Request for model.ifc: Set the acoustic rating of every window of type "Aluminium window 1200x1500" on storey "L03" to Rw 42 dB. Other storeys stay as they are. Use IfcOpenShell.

First a look at what the model holds.

```python
import ifcopenshell
import ifcopenshell.util.element

model = ifcopenshell.open("model.ifc")
print(model.schema)
storey = next(s for s in model.by_type("IfcBuildingStorey") if s.Name == "L03")
windows = [e for e in ifcopenshell.util.element.get_decomposition(storey) if e.is_a("IfcWindow")]
seen = {}
for e in windows:
    element_type = ifcopenshell.util.element.get_type(e)
    key = (element_type.Name if element_type != e and element_type else None, ifcopenshell.util.element.get_pset(e, "Pset_WindowCommon", "AcousticRating"))
    seen[key] = seen.get(key, 0) + 1
for (name, value), count in sorted(seen.items(), key=str):
    print(count, "x", name, "|", value)
```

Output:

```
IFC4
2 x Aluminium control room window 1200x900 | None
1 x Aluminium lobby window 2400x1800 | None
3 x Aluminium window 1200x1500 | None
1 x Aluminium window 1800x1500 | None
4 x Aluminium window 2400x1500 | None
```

```python
import ifcopenshell
import ifcopenshell.api.pset
import ifcopenshell.util.element

model = ifcopenshell.open("model.ifc")

storey = next(s for s in model.by_type("IfcBuildingStorey") if s.Name == "L03")
windows = [e for e in ifcopenshell.util.element.get_decomposition(storey) if e.is_a("IfcWindow")]

count = 0
for e in windows:
    element_type = ifcopenshell.util.element.get_type(e)
    if element_type in (None, e) or element_type.Name != "Aluminium window 1200x1500":
        continue
    # add_pset returns the element's existing set when there is one.
    pset = ifcopenshell.api.pset.add_pset(model, product=e, name="Pset_WindowCommon")
    ifcopenshell.api.pset.edit_pset(model, pset=pset, properties={"AcousticRating": "Rw 42 dB"})
    count += 1

print(count, "windows updated")

model.write("model_rev.ifc")
```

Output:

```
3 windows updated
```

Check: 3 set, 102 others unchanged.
